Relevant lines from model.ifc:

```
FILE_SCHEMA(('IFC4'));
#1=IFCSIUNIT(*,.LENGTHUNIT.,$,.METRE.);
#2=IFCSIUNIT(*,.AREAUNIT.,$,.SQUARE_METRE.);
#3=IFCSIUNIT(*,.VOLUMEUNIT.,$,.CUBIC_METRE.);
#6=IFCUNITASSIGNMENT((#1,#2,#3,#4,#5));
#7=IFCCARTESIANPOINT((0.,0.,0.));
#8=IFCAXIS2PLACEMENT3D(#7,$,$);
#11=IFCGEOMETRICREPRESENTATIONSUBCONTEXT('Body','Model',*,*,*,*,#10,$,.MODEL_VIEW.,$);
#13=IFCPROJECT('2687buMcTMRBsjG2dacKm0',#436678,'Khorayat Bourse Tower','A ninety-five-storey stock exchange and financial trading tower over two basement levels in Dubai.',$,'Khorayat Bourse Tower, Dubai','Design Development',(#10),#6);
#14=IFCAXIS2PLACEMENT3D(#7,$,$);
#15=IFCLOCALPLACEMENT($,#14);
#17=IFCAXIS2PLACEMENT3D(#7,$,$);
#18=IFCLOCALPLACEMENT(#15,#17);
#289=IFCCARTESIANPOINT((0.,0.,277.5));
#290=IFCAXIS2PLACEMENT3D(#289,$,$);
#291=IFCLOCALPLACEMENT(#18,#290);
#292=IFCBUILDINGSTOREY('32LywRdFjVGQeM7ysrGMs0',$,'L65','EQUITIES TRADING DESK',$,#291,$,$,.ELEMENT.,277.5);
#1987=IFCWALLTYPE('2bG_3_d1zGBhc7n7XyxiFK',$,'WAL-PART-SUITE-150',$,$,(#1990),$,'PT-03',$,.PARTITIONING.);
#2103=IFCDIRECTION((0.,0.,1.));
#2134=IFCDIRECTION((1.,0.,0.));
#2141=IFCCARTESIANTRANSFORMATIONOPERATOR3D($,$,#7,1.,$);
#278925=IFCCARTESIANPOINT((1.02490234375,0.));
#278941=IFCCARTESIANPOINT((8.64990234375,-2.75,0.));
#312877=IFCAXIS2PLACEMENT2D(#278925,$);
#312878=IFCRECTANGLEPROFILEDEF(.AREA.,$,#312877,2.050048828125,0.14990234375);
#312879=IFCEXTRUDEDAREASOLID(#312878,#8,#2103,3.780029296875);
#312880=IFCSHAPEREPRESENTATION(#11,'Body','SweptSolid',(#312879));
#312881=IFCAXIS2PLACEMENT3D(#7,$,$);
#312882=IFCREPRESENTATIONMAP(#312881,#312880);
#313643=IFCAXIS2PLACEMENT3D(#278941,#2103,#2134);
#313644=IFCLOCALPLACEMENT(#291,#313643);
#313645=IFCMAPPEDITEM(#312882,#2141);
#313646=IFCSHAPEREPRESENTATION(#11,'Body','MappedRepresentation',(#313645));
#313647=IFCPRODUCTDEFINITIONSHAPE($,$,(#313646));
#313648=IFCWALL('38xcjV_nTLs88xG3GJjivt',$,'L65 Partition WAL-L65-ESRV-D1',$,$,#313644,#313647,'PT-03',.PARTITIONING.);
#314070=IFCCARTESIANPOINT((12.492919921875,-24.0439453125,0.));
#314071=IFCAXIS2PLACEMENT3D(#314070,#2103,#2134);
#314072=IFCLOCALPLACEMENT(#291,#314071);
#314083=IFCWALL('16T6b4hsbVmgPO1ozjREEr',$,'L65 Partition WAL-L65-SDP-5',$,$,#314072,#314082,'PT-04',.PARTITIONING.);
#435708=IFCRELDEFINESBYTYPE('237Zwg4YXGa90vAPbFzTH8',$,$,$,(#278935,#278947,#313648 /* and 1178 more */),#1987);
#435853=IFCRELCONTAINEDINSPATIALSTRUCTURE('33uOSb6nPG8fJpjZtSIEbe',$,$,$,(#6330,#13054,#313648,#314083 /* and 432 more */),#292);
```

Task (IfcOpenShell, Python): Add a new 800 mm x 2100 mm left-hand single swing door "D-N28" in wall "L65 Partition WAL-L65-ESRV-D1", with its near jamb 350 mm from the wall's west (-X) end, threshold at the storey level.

```python
import numpy as np
import ifcopenshell
import ifcopenshell.api.feature
import ifcopenshell.api.geometry
import ifcopenshell.api.root
import ifcopenshell.api.spatial
import ifcopenshell.geom
import ifcopenshell.util.element
import ifcopenshell.util.placement
import ifcopenshell.util.representation
import ifcopenshell.util.shape
import ifcopenshell.util.unit

model = ifcopenshell.open("model.ifc")
unit_scale = ifcopenshell.util.unit.calculate_unit_scale(model)
settings = ifcopenshell.geom.settings()


def volume(element):
    """Net volume in cubic metres, openings subtracted."""
    shape = ifcopenshell.geom.create_shape(settings, element)
    return ifcopenshell.util.shape.get_volume(shape.geometry)


wall = model.by_guid("38xcjV_nTLs88xG3GJjivt")
storey = ifcopenshell.util.element.get_container(wall, ifc_class="IfcBuildingStorey")
context = ifcopenshell.util.representation.get_context(model, "Model", "Body", "MODEL_VIEW")
before = volume(wall)

width, height, from_end, sill = 0.8, 2.1, 0.35, 0.0  # metres

# The wall runs along its own X axis, and the end named is its -X end.
wall_shape = ifcopenshell.geom.create_shape(settings, wall)
x, y, z = ifcopenshell.util.shape.get_vertices(wall_shape.geometry).T
start = x.min() + from_end
face, thickness = float(y.min()), float(y.max() - y.min())
wall_matrix = ifcopenshell.util.placement.get_local_placement(wall.ObjectPlacement)
level = ifcopenshell.util.placement.get_local_placement(storey.ObjectPlacement)[2, 3]


def in_wall(x, y):
    """Placement at x, y metres in the wall's axes, at sill height."""
    matrix = wall_matrix.copy()
    matrix[:, 3] = wall_matrix @ np.array([x / unit_scale, y / unit_scale, 0.0, 1.0])
    matrix[2, 3] = level + sill / unit_scale
    return matrix


# Opening: a box that overshoots both wall faces by 50 mm.
opening = ifcopenshell.api.root.create_entity(model, ifc_class="IfcOpeningElement", predefined_type="OPENING")
box = ifcopenshell.api.geometry.add_wall_representation(
    model, context=context, length=width, height=height, thickness=thickness + 0.1
)
ifcopenshell.api.geometry.assign_representation(model, product=opening, representation=box)
ifcopenshell.api.geometry.edit_object_placement(model, product=opening, matrix=in_wall(start, face - 0.05), is_si=False)
ifcopenshell.api.feature.add_feature(model, feature=opening, element=wall)

door = ifcopenshell.api.root.create_entity(model, ifc_class="IfcDoor", name="D-N28", predefined_type="DOOR")
door.OverallWidth, door.OverallHeight = width / unit_scale, height / unit_scale
door.OperationType = "SINGLE_SWING_LEFT"
body = ifcopenshell.api.geometry.add_door_representation(
    model,
    context=context,
    overall_width=door.OverallWidth,
    overall_height=door.OverallHeight,
    operation_type="SINGLE_SWING_LEFT",
    lining_properties={"LiningDepth": thickness / unit_scale, "ThresholdDepth": thickness / unit_scale},
)
ifcopenshell.api.geometry.assign_representation(model, product=door, representation=body)
ifcopenshell.api.spatial.assign_container(model, products=[door], relating_structure=storey)
ifcopenshell.api.feature.add_filling(model, opening=opening, element=door)

# The lining spans the wall, so the door starts at the wall face.
ifcopenshell.api.geometry.edit_object_placement(model, product=door, matrix=in_wall(start, face), is_si=False)

after = volume(wall)

print(f"wall volume {before:.3f} -> {after:.3f} m3")

model.write("model_v2.ifc")
```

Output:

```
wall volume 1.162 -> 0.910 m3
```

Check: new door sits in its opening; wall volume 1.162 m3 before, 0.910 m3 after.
